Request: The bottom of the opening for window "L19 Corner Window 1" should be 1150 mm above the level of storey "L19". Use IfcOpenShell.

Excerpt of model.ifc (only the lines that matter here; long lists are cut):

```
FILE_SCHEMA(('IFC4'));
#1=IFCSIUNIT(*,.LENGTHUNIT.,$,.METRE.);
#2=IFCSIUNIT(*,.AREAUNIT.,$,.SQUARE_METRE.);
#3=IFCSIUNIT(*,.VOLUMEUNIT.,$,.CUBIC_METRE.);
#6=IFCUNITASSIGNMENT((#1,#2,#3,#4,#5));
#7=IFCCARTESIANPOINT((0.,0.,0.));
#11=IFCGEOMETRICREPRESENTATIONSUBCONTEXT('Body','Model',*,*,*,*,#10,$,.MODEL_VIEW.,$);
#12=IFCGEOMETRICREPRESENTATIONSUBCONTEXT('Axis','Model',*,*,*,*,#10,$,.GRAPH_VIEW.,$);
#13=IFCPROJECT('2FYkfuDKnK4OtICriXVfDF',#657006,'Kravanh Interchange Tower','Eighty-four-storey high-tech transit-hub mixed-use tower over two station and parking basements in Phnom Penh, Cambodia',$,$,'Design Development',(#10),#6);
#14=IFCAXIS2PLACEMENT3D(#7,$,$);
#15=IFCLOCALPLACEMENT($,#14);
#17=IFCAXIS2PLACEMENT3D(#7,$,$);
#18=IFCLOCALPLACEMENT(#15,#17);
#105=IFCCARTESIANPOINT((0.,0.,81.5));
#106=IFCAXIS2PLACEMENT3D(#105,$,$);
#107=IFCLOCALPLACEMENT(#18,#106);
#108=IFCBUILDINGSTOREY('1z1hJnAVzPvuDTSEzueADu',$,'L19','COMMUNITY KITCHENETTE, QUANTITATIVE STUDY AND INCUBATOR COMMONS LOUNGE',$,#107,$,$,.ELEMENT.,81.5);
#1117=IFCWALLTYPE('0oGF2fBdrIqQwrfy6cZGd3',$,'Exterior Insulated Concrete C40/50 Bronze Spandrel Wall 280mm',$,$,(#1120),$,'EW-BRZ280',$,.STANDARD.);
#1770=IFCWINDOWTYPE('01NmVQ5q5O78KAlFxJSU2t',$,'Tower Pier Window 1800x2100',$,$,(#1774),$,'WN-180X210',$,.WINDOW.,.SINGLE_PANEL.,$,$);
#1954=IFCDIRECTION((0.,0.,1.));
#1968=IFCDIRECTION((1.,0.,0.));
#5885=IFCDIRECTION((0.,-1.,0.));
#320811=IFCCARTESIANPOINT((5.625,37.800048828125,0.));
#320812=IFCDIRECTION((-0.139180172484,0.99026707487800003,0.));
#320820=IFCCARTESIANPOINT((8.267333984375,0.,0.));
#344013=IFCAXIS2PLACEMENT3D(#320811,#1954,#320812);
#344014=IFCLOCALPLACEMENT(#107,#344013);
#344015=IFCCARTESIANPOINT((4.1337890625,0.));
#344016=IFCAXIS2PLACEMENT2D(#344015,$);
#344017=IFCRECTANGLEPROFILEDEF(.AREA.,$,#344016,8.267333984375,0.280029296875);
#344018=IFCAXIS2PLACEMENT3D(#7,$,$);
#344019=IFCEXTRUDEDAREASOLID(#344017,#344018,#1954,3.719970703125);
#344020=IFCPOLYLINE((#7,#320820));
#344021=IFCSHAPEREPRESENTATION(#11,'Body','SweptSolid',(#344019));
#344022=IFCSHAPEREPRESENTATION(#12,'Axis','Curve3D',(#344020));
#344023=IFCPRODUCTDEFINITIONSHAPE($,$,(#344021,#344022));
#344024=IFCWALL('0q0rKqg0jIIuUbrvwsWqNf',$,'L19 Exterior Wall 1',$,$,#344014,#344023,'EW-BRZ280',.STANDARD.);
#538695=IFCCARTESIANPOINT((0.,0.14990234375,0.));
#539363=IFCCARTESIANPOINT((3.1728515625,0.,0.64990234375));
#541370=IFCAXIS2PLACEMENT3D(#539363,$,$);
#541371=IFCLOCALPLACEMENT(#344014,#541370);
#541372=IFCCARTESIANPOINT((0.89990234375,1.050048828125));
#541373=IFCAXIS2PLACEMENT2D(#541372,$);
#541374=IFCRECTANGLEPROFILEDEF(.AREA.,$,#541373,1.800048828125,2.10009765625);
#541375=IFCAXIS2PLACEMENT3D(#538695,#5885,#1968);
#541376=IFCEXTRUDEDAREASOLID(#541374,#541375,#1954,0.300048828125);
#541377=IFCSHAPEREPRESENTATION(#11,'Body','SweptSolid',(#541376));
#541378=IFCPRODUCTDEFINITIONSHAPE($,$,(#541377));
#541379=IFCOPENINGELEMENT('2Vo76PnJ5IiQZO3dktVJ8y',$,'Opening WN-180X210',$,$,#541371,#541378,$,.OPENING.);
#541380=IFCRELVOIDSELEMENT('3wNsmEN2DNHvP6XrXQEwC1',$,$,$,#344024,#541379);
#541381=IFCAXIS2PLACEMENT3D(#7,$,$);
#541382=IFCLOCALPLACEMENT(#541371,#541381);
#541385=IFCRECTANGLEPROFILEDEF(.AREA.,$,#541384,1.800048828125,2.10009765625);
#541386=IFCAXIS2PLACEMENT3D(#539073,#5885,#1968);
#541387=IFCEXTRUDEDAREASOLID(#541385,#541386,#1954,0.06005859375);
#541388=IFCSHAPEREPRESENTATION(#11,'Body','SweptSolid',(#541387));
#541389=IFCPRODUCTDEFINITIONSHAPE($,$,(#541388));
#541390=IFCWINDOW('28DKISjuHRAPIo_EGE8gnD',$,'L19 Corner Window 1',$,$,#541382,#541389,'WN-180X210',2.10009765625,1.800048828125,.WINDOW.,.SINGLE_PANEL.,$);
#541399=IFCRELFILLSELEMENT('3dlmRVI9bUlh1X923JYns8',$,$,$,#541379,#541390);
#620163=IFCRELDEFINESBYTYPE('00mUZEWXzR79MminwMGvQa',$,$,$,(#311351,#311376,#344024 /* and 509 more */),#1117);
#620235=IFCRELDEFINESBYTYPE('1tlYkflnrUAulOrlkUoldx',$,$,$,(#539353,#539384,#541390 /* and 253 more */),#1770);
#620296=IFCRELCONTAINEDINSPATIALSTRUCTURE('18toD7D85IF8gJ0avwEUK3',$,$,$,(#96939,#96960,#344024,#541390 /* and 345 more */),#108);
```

```python
import numpy as np
import ifcopenshell
import ifcopenshell.api.geometry
import ifcopenshell.geom
import ifcopenshell.util.element
import ifcopenshell.util.placement
import ifcopenshell.util.shape
import ifcopenshell.util.unit

model = ifcopenshell.open("model.ifc")
unit_scale = ifcopenshell.util.unit.calculate_unit_scale(model)

window = model.by_id(541390)
opening = window.FillsVoids[0].RelatingOpeningElement
storey = ifcopenshell.util.element.get_container(window, ifc_class="IfcBuildingStorey")
level = ifcopenshell.util.placement.get_local_placement(storey.ObjectPlacement)[2, 3]

# The opening's origin need not be at the sill, so measure its lowest point.
shape = ifcopenshell.geom.create_shape(ifcopenshell.geom.settings(), opening)
bottom = ifcopenshell.util.shape.get_shape_bottom_elevation(shape, shape.geometry) / unit_scale
dz = level + 1.15 - bottom

shift = np.array([0.0, 0.0, dz])
# The window is placed relative to its opening, so it follows when the opening moves.
matrix = ifcopenshell.util.placement.get_local_placement(opening.ObjectPlacement)
matrix[:3, 3] += shift
ifcopenshell.api.geometry.edit_object_placement(
    model, product=opening, matrix=matrix, is_si=False, should_transform_children=True
)

print(f"moved by {dz * unit_scale:+.3f} m")

model.write("model_edited.ifc")
```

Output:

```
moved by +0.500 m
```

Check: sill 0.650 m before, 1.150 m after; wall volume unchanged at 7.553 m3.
